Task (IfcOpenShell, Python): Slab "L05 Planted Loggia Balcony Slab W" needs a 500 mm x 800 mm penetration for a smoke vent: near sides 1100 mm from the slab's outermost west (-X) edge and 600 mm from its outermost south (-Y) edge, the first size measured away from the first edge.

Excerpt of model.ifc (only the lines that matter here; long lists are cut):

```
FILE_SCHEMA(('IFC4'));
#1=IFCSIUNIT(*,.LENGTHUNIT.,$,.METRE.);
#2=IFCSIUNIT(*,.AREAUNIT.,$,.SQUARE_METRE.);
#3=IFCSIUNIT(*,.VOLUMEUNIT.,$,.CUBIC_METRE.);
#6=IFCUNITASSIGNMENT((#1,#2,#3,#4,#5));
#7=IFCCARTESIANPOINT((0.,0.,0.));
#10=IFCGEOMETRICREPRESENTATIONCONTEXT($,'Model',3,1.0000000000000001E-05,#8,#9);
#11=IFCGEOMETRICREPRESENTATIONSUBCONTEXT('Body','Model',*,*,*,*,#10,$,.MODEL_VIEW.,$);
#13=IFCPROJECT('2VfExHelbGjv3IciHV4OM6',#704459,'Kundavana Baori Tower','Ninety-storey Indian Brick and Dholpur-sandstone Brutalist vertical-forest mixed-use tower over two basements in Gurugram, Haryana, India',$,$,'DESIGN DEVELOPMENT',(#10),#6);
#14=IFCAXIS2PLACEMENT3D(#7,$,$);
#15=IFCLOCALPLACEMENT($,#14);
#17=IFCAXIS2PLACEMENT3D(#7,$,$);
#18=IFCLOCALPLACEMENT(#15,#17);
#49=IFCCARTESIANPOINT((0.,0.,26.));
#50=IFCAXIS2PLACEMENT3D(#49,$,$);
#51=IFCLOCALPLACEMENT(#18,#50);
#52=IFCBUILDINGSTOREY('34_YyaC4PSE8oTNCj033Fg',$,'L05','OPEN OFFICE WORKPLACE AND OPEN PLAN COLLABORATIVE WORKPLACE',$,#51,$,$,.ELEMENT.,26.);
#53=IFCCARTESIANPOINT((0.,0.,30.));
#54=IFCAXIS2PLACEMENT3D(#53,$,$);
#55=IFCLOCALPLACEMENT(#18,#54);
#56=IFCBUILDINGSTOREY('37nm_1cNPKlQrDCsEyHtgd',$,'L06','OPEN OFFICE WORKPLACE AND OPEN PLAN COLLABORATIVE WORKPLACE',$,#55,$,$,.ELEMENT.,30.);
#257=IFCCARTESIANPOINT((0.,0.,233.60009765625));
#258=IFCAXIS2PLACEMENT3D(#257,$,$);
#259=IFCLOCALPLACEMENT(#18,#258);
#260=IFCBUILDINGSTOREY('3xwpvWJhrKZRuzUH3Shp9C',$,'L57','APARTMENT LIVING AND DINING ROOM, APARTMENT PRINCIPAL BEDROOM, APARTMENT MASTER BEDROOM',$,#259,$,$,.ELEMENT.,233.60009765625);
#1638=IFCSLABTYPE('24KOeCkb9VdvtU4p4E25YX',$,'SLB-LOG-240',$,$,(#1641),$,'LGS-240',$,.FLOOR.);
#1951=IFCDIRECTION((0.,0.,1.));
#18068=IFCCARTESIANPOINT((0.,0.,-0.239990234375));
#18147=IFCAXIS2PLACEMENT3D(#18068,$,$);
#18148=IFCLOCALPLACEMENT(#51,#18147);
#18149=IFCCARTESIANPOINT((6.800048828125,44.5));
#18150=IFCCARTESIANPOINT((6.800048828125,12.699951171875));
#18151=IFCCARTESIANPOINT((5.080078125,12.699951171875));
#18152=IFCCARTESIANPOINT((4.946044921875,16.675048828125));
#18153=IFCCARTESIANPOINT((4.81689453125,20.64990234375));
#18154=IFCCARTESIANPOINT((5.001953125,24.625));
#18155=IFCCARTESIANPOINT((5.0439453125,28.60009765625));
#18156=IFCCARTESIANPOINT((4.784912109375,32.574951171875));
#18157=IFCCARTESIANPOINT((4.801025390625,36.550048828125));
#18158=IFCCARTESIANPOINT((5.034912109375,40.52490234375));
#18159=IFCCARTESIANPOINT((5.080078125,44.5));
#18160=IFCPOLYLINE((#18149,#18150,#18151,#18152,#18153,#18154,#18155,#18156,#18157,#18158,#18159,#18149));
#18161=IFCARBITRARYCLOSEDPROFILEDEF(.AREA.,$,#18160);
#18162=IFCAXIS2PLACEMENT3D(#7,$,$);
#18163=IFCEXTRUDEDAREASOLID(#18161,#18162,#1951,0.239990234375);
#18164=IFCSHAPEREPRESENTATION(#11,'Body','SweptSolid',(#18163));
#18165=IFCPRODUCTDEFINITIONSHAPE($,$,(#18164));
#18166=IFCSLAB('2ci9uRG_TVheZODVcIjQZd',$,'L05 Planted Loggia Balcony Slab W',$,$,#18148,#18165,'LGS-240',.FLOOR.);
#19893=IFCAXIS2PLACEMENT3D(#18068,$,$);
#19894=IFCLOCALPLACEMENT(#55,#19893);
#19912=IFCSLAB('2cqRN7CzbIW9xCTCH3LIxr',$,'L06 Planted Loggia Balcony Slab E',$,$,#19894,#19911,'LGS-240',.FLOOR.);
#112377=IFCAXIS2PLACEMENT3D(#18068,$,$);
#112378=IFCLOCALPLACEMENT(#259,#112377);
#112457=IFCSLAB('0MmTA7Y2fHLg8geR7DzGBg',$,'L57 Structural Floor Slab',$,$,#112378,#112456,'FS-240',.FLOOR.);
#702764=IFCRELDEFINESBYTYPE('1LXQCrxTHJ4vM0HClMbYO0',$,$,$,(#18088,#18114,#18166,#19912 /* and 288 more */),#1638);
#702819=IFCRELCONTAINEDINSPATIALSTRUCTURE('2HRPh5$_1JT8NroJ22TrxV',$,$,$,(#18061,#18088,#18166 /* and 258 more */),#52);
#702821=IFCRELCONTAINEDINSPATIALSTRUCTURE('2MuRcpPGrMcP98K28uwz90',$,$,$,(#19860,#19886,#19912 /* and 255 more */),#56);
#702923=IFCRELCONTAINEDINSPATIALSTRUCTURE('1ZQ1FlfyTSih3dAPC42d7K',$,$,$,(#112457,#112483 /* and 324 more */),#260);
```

```python
import numpy as np
import ifcopenshell
import ifcopenshell.api.feature
import ifcopenshell.api.geometry
import ifcopenshell.api.root
import ifcopenshell.geom
import ifcopenshell.util.placement
import ifcopenshell.util.representation
import ifcopenshell.util.shape
import ifcopenshell.util.unit

model = ifcopenshell.open("model.ifc")
unit_scale = ifcopenshell.util.unit.calculate_unit_scale(model)
settings = ifcopenshell.geom.settings()


def volume(element):
    """Net volume in cubic metres, openings subtracted."""
    shape = ifcopenshell.geom.create_shape(settings, element)
    return ifcopenshell.util.shape.get_volume(shape.geometry)


slab = model.by_guid("2ci9uRG_TVheZODVcIjQZd")
before = volume(slab)

# Extent in the slab's own axes, in metres. The edges named are its -X and -Y sides.
slab_shape = ifcopenshell.geom.create_shape(settings, slab)
vertices = ifcopenshell.util.shape.get_vertices(slab_shape.geometry)
x_min, y_min, bottom = vertices.min(axis=0)
top = vertices[:, 2].max()

opening = ifcopenshell.api.root.create_entity(model, ifc_class="IfcOpeningElement", name="Smoke vent opening", predefined_type="OPENING")
context = ifcopenshell.util.representation.get_context(model, "Model", "Body", "MODEL_VIEW")
width, depth = 0.5, 0.8
outline = [(0.0, 0.0), (width, 0.0), (width, depth), (0.0, depth), (0.0, 0.0)]
# Overshoot both faces by 50 mm so the cut is clean.
shape = ifcopenshell.api.geometry.add_slab_representation(
    model, context=context, depth=top - bottom + 0.1, polyline=outline
)
ifcopenshell.api.geometry.assign_representation(model, product=opening, representation=shape)

matrix = ifcopenshell.util.placement.get_local_placement(slab.ObjectPlacement)
matrix[:, 3] = matrix @ np.append(np.array([x_min + 1.1, y_min + 0.6, bottom - 0.05]) / unit_scale, 1.0)
ifcopenshell.api.geometry.edit_object_placement(model, product=opening, matrix=matrix, is_si=False)
ifcopenshell.api.feature.add_feature(model, feature=opening, element=slab)

after = volume(slab)

print(f"slab volume {before:.3f} -> {after:.3f} m3")

model.write("model_rev.ifc")
```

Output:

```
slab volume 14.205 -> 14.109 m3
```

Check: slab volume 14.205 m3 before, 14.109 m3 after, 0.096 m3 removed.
